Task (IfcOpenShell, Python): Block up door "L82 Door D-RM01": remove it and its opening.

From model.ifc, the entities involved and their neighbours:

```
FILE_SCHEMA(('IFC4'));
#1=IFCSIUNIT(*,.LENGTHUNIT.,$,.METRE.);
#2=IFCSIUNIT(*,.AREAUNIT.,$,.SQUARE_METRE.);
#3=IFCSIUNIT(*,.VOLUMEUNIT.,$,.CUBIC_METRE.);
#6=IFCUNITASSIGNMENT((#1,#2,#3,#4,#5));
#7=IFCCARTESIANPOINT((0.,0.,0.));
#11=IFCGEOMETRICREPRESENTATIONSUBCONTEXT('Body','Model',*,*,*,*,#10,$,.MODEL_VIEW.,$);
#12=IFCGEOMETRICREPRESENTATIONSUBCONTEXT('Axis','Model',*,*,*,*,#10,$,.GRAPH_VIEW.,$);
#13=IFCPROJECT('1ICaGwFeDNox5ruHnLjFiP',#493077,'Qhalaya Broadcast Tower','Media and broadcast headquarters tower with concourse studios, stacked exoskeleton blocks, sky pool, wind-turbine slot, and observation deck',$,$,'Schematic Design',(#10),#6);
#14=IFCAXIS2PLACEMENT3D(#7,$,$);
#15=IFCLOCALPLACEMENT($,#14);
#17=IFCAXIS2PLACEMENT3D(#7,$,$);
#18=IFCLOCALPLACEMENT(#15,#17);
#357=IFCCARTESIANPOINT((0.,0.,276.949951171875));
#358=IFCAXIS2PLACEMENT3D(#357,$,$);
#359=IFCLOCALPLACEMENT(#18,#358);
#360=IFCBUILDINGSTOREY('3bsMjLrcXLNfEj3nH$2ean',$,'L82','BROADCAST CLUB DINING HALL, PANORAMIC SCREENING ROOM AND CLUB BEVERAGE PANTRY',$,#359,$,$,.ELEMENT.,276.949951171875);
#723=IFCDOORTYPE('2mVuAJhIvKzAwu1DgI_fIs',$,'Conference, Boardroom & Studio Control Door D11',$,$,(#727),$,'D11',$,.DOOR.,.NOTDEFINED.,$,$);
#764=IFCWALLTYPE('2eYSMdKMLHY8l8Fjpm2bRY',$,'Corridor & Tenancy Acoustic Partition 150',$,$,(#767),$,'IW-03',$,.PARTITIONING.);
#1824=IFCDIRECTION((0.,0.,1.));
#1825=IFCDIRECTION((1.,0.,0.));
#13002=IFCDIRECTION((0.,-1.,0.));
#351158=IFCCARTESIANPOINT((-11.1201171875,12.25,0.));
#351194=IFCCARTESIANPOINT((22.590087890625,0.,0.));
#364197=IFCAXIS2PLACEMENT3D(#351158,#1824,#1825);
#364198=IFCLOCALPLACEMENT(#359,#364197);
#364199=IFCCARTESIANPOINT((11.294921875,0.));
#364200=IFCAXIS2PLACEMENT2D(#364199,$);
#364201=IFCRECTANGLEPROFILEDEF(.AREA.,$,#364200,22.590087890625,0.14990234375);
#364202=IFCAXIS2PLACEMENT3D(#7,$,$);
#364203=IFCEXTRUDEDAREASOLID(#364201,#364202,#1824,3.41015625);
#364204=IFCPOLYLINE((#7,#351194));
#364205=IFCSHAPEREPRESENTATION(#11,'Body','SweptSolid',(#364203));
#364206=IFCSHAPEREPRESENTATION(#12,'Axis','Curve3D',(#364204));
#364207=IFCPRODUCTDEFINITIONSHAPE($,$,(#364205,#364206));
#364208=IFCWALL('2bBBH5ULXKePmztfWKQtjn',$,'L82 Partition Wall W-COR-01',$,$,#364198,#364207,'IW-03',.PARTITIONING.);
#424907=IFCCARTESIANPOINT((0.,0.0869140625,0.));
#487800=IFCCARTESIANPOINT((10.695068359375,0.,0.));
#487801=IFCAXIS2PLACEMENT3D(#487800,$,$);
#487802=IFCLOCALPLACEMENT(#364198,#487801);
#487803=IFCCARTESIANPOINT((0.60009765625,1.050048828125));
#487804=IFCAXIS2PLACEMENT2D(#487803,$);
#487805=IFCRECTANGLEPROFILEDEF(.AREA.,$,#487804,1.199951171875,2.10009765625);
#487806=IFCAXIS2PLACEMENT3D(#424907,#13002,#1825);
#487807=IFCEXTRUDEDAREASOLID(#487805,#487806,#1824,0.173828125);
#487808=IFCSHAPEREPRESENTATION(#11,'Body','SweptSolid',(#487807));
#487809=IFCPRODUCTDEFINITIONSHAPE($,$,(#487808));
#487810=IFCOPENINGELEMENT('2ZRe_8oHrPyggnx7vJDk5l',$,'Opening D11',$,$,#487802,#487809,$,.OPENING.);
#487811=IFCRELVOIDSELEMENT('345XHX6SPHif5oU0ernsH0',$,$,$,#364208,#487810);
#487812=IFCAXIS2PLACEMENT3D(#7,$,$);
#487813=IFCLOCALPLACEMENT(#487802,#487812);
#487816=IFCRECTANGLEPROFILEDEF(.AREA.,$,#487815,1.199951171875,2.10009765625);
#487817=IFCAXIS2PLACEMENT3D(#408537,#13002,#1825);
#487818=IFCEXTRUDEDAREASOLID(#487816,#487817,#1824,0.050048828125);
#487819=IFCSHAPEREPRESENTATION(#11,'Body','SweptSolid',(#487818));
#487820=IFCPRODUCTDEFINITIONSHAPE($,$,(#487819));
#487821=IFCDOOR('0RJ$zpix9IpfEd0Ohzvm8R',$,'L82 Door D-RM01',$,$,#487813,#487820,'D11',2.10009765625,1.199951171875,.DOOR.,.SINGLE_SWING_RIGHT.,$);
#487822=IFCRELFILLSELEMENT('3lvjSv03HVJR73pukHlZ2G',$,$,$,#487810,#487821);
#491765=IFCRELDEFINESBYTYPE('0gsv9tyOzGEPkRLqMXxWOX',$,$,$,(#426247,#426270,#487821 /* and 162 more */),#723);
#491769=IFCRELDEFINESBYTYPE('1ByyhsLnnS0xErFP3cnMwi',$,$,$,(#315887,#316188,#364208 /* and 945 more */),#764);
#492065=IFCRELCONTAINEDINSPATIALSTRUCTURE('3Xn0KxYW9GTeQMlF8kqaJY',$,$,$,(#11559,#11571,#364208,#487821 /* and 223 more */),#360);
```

```python
import ifcopenshell
import ifcopenshell.api.feature
import ifcopenshell.api.root
import ifcopenshell.geom
import ifcopenshell.util.shape

model = ifcopenshell.open("model.ifc")
settings = ifcopenshell.geom.settings()


def volume(element):
    """Net volume in cubic metres, openings subtracted."""
    shape = ifcopenshell.geom.create_shape(settings, element)
    return ifcopenshell.util.shape.get_volume(shape.geometry)


door = model.by_guid("0RJ$zpix9IpfEd0Ohzvm8R")
opening = door.FillsVoids[0].RelatingOpeningElement
wall = opening.VoidsElements[0].RelatingBuildingElement
before = volume(wall)

ifcopenshell.api.root.remove_product(model, product=door)
ifcopenshell.api.feature.remove_feature(model, feature=opening)

after = volume(wall)

print(f"wall volume {before:.3f} -> {after:.3f} m3")

model.write("model_v2.ifc")
```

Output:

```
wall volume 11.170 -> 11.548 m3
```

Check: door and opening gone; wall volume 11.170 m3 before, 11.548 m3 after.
